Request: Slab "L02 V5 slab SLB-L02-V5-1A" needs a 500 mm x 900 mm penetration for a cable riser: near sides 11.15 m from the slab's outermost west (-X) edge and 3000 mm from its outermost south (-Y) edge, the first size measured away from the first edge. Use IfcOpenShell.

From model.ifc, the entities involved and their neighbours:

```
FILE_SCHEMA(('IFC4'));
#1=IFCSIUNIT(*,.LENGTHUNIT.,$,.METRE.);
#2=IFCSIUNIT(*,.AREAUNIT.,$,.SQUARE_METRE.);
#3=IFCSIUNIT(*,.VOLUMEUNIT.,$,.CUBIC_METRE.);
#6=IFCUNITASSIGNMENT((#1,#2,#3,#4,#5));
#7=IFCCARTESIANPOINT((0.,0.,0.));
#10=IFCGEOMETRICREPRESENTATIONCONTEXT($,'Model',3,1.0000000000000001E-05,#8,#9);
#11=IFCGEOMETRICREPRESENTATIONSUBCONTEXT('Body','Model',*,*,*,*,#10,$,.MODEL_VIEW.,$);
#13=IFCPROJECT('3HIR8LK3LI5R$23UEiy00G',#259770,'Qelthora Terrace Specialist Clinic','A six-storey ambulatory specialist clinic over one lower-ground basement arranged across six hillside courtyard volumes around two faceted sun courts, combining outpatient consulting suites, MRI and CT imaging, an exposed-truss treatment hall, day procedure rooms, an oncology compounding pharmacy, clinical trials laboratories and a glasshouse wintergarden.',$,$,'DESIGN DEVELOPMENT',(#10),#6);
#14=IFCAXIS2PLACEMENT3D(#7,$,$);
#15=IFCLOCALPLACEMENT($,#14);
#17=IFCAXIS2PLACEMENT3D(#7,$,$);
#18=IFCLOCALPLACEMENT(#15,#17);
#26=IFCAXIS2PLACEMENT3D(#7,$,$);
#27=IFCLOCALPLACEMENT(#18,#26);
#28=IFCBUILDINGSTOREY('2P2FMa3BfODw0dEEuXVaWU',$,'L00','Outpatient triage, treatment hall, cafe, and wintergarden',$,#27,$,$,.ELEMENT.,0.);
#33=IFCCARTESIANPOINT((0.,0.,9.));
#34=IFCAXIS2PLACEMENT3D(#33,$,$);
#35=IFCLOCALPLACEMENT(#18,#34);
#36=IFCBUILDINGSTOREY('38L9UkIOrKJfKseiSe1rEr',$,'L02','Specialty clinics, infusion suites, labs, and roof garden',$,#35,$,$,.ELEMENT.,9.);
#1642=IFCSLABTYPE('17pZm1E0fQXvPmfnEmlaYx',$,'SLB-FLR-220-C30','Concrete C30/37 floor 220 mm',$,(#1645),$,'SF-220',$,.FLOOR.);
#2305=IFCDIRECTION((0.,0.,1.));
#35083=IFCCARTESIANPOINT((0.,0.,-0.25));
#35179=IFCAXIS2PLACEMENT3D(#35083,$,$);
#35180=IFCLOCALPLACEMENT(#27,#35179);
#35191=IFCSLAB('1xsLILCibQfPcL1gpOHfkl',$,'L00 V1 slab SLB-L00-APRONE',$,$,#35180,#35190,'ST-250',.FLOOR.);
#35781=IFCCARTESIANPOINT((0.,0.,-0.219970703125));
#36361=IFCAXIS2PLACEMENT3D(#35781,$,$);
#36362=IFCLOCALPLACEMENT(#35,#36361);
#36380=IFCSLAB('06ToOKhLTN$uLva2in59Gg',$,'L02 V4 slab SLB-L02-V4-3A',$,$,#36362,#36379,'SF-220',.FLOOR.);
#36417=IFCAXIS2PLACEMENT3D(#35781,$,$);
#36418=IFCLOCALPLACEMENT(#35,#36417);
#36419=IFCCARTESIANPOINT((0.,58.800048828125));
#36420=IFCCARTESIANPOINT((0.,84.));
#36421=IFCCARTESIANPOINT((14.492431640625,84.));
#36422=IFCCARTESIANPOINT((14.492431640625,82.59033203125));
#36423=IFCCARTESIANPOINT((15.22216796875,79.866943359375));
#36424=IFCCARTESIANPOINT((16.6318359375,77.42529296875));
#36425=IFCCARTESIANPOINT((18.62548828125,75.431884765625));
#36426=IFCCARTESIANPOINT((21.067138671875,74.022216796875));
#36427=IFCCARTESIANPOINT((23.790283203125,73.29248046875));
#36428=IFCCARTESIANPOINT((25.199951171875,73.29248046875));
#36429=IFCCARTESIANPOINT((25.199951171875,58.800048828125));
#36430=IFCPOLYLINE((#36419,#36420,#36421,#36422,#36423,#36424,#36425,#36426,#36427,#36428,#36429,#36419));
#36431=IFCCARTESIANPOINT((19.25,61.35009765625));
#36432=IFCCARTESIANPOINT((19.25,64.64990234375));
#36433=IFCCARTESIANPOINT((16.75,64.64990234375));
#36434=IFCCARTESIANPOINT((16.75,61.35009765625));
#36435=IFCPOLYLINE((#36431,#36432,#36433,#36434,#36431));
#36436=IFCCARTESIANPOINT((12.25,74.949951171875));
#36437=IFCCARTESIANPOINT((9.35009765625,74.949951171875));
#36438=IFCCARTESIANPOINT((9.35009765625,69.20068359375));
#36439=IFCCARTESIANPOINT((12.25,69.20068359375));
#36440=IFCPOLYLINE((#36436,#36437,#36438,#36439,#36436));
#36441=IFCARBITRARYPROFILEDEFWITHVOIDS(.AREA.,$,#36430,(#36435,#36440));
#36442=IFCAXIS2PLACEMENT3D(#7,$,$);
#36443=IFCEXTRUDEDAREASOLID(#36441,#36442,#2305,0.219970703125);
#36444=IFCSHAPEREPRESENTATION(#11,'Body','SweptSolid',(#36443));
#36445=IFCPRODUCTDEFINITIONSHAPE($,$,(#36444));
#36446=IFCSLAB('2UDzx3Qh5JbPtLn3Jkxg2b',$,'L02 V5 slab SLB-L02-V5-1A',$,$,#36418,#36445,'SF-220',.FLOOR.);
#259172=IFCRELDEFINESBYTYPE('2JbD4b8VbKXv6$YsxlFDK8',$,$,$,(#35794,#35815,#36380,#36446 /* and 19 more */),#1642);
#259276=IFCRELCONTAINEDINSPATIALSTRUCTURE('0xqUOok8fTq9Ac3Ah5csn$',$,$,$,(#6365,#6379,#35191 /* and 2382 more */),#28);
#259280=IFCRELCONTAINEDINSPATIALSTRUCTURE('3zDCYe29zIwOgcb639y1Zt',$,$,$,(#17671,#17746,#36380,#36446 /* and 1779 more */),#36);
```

```python
import numpy as np
import ifcopenshell
import ifcopenshell.api.feature
import ifcopenshell.api.geometry
import ifcopenshell.api.root
import ifcopenshell.geom
import ifcopenshell.util.placement
import ifcopenshell.util.representation
import ifcopenshell.util.shape
import ifcopenshell.util.unit

model = ifcopenshell.open("model.ifc")
unit_scale = ifcopenshell.util.unit.calculate_unit_scale(model)
settings = ifcopenshell.geom.settings()


def volume(element):
    """Net volume in cubic metres, openings subtracted."""
    shape = ifcopenshell.geom.create_shape(settings, element)
    return ifcopenshell.util.shape.get_volume(shape.geometry)


slab = model.by_id(36446)
before = volume(slab)

# Extent in the slab's own axes, in metres. The edges named are its -X and -Y sides.
slab_shape = ifcopenshell.geom.create_shape(settings, slab)
vertices = ifcopenshell.util.shape.get_vertices(slab_shape.geometry)
x_min, y_min, bottom = vertices.min(axis=0)
top = vertices[:, 2].max()

opening = ifcopenshell.api.root.create_entity(model, ifc_class="IfcOpeningElement", name="Cable riser opening", predefined_type="OPENING")
context = ifcopenshell.util.representation.get_context(model, "Model", "Body", "MODEL_VIEW")
width, depth = 0.5, 0.9
outline = [(0.0, 0.0), (width, 0.0), (width, depth), (0.0, depth), (0.0, 0.0)]
# Overshoot both faces by 50 mm so the cut is clean.
shape = ifcopenshell.api.geometry.add_slab_representation(
    model, context=context, depth=top - bottom + 0.1, polyline=outline
)
ifcopenshell.api.geometry.assign_representation(model, product=opening, representation=shape)

matrix = ifcopenshell.util.placement.get_local_placement(slab.ObjectPlacement)
matrix[:, 3] = matrix @ np.append(np.array([x_min + 11.15, y_min + 3, bottom - 0.05]) / unit_scale, 1.0)
ifcopenshell.api.geometry.edit_object_placement(model, product=opening, matrix=matrix, is_si=False)
ifcopenshell.api.feature.add_feature(model, feature=opening, element=slab)

after = volume(slab)

print(f"slab volume {before:.3f} -> {after:.3f} m3")

model.write("model-out.ifc")
```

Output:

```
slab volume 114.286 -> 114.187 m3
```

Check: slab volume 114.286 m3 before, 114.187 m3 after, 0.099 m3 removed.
